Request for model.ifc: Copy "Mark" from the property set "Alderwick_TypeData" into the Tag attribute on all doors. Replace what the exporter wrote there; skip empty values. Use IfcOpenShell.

First a look at what the model holds.

```python
import ifcopenshell
import ifcopenshell.util.element

model = ifcopenshell.open("model.ifc")
print(model.schema)
doors = model.by_type("IfcDoor")
print(len(doors), "doors")
for e in doors[:8]:
    source = ifcopenshell.util.element.get_pset(e, "Alderwick_TypeData", "Mark")
    target = e.Tag
    print(e.id(), repr(source), repr(target), sep=" | ")
```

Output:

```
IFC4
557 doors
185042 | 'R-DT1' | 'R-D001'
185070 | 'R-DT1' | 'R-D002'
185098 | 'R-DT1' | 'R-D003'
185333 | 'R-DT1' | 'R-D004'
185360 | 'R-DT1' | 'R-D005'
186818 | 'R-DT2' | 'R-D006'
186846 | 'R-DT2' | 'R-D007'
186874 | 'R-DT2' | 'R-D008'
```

```python
import ifcopenshell
import ifcopenshell.util.element

model = ifcopenshell.open("model.ifc")

count = 0
for e in model.by_type("IfcDoor"):
    value = ifcopenshell.util.element.get_pset(e, "Alderwick_TypeData", "Mark")
    current = e.Tag
    if not value or not value.strip() or current == value:
        continue
    e.Tag = value
    count += 1

print(count, "doors updated")

model.write("model_v2.ifc")
```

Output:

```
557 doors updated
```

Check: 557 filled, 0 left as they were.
